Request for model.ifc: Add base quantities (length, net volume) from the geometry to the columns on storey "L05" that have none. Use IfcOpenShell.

First a look at what the model holds.

```python
import ifcopenshell
import ifcopenshell.util.element
import ifcopenshell.util.unit

model = ifcopenshell.open("model.ifc")
print(model.schema)
for unit_type in ("LENGTHUNIT", "AREAUNIT", "VOLUMEUNIT"):
    print(unit_type, ifcopenshell.util.unit.calculate_unit_scale(model, unit_type))
storey = next(s for s in model.by_type("IfcBuildingStorey") if s.Name == "L05")
columns = [e for e in ifcopenshell.util.element.get_decomposition(storey) if e.is_a("IfcColumn")]
for e in sorted(columns, key=lambda e: e.id()):
    print(e.id(), e.is_a(), e.Name, list(ifcopenshell.util.element.get_psets(e, qtos_only=True)), sep=" | ")
```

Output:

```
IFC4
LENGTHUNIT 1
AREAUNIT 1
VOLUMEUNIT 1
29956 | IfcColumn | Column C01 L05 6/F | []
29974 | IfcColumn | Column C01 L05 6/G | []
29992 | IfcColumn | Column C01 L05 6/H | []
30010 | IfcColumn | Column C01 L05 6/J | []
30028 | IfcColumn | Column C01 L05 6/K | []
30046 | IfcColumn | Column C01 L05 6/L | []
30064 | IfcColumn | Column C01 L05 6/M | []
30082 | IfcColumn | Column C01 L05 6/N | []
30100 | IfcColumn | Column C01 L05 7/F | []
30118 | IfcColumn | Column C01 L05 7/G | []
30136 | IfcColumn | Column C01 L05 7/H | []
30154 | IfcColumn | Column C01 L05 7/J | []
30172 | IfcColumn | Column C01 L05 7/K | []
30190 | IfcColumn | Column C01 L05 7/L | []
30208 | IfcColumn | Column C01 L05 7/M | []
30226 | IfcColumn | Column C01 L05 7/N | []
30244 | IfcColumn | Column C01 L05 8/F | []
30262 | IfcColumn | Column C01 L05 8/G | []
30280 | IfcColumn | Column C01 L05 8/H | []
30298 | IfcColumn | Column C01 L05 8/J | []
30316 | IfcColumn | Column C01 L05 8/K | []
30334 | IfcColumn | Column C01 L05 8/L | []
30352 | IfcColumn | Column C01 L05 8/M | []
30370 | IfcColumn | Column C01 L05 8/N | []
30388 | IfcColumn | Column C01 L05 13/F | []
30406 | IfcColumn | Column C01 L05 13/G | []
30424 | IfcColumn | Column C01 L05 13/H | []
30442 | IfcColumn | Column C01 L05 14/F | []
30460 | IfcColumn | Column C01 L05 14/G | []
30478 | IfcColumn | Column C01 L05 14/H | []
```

```python
import ifcopenshell
import ifcopenshell.api.pset
import ifcopenshell.geom
import ifcopenshell.util.element
import ifcopenshell.util.shape
import ifcopenshell.util.unit

model = ifcopenshell.open("model.ifc")
unit_scale = ifcopenshell.util.unit.calculate_unit_scale(model)
volume_scale = ifcopenshell.util.unit.calculate_unit_scale(model, "VOLUMEUNIT")
settings = ifcopenshell.geom.settings()

storey = next(s for s in model.by_type("IfcBuildingStorey") if s.Name == "L05")
columns = [e for e in ifcopenshell.util.element.get_decomposition(storey) if e.is_a("IfcColumn")]

for e in sorted(columns, key=lambda e: e.id()):
    if ifcopenshell.util.element.get_psets(e, qtos_only=True, should_inherit=False):
        continue
    # Geometry comes back in metres, in the element's own axes.
    shape = ifcopenshell.geom.create_shape(settings, e)
    values = {
        "Length": ifcopenshell.util.shape.get_z(shape.geometry) / unit_scale,
        "NetVolume": ifcopenshell.util.shape.get_volume(shape.geometry) / volume_scale,
    }
    qto = ifcopenshell.api.pset.add_qto(model, product=e, name="Qto_ColumnBaseQuantities")
    ifcopenshell.api.pset.edit_qto(model, qto=qto, properties=values)
    print(e.id(), {k: round(v, 3) for k, v in values.items()})

model.write("model_v2.ifc")
```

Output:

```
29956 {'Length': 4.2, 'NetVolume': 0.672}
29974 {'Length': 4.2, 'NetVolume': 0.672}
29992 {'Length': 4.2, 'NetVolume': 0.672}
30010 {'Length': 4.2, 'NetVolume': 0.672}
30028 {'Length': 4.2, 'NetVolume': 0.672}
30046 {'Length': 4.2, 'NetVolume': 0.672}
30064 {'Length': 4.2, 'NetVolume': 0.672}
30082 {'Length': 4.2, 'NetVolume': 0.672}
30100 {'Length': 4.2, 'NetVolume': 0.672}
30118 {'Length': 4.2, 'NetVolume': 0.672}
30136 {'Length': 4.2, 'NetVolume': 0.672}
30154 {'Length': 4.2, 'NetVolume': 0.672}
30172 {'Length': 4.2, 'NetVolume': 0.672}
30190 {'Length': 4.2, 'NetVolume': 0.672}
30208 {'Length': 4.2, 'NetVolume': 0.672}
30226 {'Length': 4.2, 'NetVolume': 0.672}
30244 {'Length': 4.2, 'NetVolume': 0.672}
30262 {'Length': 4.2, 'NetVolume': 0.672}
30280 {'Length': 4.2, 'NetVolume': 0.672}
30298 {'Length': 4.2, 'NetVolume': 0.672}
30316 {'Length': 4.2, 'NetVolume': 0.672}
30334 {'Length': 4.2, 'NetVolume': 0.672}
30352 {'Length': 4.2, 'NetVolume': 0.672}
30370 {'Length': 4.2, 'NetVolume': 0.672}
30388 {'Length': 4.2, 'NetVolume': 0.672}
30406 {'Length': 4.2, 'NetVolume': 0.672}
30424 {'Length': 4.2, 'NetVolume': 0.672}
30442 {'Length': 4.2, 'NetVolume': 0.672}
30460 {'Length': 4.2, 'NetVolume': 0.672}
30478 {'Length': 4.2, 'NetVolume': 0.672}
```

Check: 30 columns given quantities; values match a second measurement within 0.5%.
